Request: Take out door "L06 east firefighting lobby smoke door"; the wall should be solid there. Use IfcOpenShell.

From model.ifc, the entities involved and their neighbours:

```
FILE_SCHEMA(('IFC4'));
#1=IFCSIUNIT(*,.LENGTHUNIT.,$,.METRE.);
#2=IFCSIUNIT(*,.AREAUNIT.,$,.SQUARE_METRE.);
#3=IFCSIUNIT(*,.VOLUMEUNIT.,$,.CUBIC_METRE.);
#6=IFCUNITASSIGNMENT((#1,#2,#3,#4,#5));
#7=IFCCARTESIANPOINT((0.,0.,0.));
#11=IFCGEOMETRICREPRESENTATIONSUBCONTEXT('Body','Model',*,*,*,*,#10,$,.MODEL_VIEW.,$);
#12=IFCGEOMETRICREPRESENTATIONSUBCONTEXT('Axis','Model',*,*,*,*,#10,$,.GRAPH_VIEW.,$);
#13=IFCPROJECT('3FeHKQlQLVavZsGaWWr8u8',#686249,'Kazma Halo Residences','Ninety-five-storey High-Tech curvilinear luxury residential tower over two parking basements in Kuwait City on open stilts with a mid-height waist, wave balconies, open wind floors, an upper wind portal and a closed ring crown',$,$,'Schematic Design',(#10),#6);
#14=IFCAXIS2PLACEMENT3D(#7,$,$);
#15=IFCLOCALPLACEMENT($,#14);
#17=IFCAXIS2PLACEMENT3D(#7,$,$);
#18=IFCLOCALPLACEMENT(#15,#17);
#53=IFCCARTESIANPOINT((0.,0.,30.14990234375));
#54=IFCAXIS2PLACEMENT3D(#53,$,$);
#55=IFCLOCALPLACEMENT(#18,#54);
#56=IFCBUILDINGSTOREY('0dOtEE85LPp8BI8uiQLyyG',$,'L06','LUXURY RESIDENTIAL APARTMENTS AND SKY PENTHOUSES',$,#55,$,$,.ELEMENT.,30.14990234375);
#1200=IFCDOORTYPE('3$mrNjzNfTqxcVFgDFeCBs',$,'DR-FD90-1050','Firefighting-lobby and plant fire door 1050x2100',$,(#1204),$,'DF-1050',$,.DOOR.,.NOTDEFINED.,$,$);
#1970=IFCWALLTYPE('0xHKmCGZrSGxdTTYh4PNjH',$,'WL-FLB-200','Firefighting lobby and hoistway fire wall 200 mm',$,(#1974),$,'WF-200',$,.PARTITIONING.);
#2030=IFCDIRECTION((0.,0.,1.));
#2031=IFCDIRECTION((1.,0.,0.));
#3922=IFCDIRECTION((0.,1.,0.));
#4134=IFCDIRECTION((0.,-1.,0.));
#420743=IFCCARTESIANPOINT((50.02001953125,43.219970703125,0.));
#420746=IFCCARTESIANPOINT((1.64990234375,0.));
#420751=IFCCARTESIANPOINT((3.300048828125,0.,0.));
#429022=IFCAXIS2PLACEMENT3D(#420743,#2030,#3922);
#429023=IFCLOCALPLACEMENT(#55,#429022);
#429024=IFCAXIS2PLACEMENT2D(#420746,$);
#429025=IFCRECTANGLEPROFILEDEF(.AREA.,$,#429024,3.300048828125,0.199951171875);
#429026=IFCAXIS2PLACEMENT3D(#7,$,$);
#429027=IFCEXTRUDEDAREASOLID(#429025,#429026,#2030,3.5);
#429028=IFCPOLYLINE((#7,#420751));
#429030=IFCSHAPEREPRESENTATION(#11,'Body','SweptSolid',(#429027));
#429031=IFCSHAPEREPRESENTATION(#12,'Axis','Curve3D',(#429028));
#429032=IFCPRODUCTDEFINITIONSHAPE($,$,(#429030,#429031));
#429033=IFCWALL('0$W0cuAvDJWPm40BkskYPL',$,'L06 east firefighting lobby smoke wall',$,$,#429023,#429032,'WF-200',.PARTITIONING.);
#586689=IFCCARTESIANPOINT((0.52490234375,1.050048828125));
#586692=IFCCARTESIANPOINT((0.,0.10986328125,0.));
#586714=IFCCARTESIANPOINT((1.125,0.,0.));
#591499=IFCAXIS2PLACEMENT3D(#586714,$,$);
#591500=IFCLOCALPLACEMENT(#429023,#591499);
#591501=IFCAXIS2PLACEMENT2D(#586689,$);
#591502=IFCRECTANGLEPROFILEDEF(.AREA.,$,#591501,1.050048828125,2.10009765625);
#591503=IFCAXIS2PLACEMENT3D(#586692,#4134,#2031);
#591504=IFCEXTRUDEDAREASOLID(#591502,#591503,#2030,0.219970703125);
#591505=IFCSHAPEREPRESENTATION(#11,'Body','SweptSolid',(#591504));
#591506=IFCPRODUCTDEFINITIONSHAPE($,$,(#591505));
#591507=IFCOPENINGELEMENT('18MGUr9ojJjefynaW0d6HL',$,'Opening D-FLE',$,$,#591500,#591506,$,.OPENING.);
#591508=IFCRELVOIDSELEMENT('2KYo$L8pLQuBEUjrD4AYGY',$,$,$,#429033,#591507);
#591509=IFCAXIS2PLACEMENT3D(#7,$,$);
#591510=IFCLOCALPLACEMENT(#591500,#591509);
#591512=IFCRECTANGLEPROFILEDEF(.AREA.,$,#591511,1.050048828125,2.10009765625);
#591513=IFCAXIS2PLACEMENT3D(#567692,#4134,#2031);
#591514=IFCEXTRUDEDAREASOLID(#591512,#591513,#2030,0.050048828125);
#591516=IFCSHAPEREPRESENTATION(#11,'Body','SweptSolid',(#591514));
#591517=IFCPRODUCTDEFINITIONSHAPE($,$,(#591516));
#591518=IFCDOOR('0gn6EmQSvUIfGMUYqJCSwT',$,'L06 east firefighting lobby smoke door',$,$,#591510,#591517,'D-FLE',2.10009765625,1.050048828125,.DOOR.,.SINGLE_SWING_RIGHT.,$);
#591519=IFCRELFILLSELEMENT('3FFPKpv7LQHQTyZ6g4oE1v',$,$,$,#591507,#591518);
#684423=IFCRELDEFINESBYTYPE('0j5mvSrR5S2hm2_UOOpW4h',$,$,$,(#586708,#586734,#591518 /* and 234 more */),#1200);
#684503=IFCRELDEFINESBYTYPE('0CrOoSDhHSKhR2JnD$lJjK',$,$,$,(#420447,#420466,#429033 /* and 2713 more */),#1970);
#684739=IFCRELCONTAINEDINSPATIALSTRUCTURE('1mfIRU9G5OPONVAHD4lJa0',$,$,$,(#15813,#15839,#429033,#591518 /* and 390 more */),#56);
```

```python
import ifcopenshell
import ifcopenshell.api.feature
import ifcopenshell.api.root
import ifcopenshell.geom
import ifcopenshell.util.shape

model = ifcopenshell.open("model.ifc")
settings = ifcopenshell.geom.settings()


def volume(element):
    """Net volume in cubic metres, openings subtracted."""
    shape = ifcopenshell.geom.create_shape(settings, element)
    return ifcopenshell.util.shape.get_volume(shape.geometry)


door = model.by_guid("0gn6EmQSvUIfGMUYqJCSwT")
opening = door.FillsVoids[0].RelatingOpeningElement
wall = opening.VoidsElements[0].RelatingBuildingElement
before = volume(wall)

ifcopenshell.api.root.remove_product(model, product=door)
ifcopenshell.api.feature.remove_feature(model, feature=opening)

after = volume(wall)

print(f"wall volume {before:.3f} -> {after:.3f} m3")

model.write("model_v2.ifc")
```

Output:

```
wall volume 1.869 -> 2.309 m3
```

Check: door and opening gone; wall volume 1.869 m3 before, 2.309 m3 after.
